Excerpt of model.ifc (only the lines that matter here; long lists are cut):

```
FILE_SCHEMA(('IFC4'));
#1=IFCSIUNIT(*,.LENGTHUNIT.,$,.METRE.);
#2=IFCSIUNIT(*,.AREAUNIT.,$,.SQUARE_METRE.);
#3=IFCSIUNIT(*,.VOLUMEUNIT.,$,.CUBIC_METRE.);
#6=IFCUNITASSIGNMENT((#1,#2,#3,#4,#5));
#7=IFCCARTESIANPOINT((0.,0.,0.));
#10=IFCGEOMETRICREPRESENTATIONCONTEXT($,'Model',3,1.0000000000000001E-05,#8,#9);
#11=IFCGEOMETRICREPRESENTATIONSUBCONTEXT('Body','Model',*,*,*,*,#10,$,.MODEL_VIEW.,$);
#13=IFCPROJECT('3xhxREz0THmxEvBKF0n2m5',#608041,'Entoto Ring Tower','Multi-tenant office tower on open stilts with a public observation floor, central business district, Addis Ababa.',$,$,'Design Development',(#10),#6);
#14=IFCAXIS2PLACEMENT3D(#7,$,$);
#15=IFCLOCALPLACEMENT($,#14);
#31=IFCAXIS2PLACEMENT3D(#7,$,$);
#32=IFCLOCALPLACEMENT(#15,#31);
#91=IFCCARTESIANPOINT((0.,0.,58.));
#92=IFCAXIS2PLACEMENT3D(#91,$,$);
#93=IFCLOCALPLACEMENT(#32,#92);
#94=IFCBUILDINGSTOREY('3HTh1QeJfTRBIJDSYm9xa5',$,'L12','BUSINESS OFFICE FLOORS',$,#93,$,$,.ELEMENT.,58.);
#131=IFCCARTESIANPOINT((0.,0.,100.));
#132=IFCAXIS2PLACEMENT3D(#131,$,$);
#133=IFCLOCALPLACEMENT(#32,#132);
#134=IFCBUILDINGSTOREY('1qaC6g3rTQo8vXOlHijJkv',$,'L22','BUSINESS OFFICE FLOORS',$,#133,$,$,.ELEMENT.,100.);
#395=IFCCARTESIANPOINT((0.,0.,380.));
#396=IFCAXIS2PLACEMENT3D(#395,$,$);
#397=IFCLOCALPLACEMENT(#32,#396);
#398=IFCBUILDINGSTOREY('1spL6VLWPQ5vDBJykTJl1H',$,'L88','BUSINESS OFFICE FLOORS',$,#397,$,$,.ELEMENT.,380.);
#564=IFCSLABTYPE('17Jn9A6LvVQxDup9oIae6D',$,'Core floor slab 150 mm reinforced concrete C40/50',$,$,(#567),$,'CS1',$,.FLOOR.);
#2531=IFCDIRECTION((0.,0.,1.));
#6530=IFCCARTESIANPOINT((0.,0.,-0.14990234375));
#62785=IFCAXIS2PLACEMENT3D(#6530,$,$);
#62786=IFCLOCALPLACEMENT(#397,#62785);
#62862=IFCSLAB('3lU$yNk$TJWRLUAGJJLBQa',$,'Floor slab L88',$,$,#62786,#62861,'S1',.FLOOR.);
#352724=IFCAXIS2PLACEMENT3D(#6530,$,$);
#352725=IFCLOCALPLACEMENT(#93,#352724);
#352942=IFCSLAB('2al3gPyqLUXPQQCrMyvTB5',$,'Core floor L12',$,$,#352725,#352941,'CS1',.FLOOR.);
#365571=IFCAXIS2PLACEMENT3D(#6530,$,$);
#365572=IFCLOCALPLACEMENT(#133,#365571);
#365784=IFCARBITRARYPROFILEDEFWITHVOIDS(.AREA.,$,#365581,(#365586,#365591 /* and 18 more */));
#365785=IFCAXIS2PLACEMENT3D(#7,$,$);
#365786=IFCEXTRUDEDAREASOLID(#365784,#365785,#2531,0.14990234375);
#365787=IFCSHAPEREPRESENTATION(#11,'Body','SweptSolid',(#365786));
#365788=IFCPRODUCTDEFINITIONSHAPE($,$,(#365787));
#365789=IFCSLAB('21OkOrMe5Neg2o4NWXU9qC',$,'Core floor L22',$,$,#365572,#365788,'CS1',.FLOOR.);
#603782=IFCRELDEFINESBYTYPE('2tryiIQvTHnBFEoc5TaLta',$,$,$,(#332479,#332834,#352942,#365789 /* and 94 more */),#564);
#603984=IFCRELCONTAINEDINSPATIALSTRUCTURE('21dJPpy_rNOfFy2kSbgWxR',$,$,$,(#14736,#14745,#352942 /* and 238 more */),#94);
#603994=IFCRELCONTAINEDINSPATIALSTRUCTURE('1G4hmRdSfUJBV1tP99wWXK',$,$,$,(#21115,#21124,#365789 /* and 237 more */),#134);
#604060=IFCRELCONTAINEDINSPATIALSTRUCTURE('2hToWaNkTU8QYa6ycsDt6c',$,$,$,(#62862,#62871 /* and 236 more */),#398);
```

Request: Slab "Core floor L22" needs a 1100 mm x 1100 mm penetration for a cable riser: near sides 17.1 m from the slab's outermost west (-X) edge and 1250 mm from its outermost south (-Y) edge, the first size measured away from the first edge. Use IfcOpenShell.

```python
import numpy as np
import ifcopenshell
import ifcopenshell.api.feature
import ifcopenshell.api.geometry
import ifcopenshell.api.root
import ifcopenshell.geom
import ifcopenshell.util.placement
import ifcopenshell.util.representation
import ifcopenshell.util.shape
import ifcopenshell.util.unit

model = ifcopenshell.open("model.ifc")
unit_scale = ifcopenshell.util.unit.calculate_unit_scale(model)
settings = ifcopenshell.geom.settings()


def volume(element):
    """Net volume in cubic metres, openings subtracted."""
    shape = ifcopenshell.geom.create_shape(settings, element)
    return ifcopenshell.util.shape.get_volume(shape.geometry)


slab = model.by_id(365789)
before = volume(slab)

# Extent in the slab's own axes, in metres. The edges named are its -X and -Y sides.
slab_shape = ifcopenshell.geom.create_shape(settings, slab)
vertices = ifcopenshell.util.shape.get_vertices(slab_shape.geometry)
x_min, y_min, bottom = vertices.min(axis=0)
top = vertices[:, 2].max()

opening = ifcopenshell.api.root.create_entity(model, ifc_class="IfcOpeningElement", name="Cable riser opening", predefined_type="OPENING")
context = ifcopenshell.util.representation.get_context(model, "Model", "Body", "MODEL_VIEW")
width, depth = 1.1, 1.1
outline = [(0.0, 0.0), (width, 0.0), (width, depth), (0.0, depth), (0.0, 0.0)]
# Overshoot both faces by 50 mm so the cut is clean.
shape = ifcopenshell.api.geometry.add_slab_representation(
    model, context=context, depth=top - bottom + 0.1, polyline=outline
)
ifcopenshell.api.geometry.assign_representation(model, product=opening, representation=shape)

matrix = ifcopenshell.util.placement.get_local_placement(slab.ObjectPlacement)
matrix[:, 3] = matrix @ np.append(np.array([x_min + 17.1, y_min + 1.25, bottom - 0.05]) / unit_scale, 1.0)
ifcopenshell.api.geometry.edit_object_placement(model, product=opening, matrix=matrix, is_si=False)
ifcopenshell.api.feature.add_feature(model, feature=opening, element=slab)

after = volume(slab)

print(f"slab volume {before:.3f} -> {after:.3f} m3")

model.write("model_v2.ifc")
```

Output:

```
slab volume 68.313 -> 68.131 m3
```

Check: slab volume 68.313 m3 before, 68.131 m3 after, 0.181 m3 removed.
